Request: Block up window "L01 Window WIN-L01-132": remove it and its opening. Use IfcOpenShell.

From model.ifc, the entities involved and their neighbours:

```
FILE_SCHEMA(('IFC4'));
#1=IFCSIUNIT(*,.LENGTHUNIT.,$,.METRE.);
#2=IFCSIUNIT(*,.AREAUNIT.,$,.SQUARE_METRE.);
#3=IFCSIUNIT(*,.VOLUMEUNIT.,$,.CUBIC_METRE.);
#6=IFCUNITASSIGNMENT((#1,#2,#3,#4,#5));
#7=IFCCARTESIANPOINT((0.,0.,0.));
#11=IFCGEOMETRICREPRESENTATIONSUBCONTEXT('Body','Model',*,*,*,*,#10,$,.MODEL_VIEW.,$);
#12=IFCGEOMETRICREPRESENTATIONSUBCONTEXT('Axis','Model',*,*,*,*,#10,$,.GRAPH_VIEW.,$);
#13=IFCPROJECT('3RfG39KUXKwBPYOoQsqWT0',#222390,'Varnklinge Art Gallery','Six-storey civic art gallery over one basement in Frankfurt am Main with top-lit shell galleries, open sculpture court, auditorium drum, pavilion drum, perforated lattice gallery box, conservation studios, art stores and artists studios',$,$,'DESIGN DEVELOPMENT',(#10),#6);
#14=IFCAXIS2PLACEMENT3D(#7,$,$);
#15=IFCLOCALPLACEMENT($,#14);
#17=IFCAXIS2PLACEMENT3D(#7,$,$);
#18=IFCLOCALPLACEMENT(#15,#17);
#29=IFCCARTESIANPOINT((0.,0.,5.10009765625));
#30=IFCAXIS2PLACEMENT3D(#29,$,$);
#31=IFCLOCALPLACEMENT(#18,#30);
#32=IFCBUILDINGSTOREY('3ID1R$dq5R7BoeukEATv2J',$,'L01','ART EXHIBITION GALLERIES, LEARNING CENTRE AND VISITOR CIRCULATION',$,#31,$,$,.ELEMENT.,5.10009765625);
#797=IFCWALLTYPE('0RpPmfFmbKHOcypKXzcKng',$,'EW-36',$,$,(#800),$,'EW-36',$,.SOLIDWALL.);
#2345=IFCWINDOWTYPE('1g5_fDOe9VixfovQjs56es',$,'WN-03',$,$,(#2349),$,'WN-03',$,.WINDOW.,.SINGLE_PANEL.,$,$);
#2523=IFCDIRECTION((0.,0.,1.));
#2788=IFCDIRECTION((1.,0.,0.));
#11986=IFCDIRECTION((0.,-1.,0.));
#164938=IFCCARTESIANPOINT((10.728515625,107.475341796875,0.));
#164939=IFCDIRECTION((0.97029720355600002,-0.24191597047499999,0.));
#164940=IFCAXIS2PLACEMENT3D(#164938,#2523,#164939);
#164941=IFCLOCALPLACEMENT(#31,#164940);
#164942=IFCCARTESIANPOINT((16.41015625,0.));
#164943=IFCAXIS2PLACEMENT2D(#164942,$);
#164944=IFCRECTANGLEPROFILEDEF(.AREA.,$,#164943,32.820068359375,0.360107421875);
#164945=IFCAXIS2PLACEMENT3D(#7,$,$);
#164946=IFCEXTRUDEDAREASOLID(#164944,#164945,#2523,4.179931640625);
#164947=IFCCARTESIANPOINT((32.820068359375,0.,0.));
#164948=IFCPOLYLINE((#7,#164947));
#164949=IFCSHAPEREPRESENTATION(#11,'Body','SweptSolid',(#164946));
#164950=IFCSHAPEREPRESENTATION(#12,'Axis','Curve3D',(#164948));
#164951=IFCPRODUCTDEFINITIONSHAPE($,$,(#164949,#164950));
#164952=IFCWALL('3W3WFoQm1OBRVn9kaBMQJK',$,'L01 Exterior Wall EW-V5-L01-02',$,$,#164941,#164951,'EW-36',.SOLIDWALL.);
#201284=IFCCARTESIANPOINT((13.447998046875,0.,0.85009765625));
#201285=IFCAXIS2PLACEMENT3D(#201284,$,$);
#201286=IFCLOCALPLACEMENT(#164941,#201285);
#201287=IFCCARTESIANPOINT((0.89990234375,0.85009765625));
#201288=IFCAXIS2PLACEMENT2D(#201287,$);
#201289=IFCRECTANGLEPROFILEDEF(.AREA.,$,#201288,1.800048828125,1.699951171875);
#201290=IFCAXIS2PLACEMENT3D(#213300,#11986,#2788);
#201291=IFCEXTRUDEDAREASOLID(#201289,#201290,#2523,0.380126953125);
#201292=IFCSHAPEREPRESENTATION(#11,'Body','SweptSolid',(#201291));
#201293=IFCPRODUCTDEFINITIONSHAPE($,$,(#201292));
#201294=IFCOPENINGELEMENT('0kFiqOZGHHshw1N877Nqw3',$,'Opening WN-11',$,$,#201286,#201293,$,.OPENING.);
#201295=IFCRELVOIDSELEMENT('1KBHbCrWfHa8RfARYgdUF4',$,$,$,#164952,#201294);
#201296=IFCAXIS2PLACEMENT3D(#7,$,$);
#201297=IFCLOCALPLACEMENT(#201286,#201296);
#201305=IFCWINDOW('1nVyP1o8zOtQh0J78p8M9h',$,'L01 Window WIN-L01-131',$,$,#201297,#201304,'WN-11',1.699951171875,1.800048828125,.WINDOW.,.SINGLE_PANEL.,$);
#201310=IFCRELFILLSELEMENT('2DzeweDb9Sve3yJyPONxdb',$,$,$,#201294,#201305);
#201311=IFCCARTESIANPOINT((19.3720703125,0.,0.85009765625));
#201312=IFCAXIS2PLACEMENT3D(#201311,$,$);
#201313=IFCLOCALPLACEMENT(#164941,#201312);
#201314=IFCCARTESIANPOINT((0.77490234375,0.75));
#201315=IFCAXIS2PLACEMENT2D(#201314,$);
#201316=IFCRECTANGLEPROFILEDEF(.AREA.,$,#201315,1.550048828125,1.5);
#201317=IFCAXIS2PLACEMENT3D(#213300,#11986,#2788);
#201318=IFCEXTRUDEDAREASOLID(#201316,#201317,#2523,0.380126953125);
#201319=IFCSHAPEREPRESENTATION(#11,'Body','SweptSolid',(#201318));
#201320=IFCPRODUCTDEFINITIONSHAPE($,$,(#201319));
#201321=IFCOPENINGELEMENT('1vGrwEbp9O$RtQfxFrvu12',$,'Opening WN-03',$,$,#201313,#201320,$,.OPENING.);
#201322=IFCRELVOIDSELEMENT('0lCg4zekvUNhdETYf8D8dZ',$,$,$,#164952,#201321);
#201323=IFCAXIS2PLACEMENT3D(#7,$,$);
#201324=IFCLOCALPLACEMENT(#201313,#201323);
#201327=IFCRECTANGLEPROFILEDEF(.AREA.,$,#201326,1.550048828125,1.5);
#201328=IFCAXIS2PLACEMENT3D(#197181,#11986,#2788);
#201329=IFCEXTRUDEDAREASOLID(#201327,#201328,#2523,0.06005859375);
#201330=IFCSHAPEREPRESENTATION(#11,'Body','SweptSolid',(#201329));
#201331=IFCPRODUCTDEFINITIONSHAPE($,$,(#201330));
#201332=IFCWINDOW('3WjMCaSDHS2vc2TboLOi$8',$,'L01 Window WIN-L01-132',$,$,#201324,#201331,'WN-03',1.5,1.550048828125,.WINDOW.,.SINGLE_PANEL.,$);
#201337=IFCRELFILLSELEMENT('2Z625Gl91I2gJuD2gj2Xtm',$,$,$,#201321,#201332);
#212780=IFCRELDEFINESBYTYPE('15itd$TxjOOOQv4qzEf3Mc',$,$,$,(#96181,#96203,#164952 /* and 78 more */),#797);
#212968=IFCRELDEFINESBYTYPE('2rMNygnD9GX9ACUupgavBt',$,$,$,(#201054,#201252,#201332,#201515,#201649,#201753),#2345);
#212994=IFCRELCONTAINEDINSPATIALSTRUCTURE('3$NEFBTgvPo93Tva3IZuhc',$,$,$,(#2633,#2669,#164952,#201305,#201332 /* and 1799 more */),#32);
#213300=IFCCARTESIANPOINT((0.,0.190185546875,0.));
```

```python
import ifcopenshell
import ifcopenshell.api.feature
import ifcopenshell.api.root
import ifcopenshell.geom
import ifcopenshell.util.shape

model = ifcopenshell.open("model.ifc")
settings = ifcopenshell.geom.settings()


def volume(element):
    """Net volume in cubic metres, openings subtracted."""
    shape = ifcopenshell.geom.create_shape(settings, element)
    return ifcopenshell.util.shape.get_volume(shape.geometry)


window = model.by_guid("3WjMCaSDHS2vc2TboLOi$8")
opening = window.FillsVoids[0].RelatingOpeningElement
wall = opening.VoidsElements[0].RelatingBuildingElement
before = volume(wall)

ifcopenshell.api.root.remove_product(model, product=window)
ifcopenshell.api.feature.remove_feature(model, feature=opening)

after = volume(wall)

print(f"wall volume {before:.3f} -> {after:.3f} m3")

model.write("model_v2.ifc")
```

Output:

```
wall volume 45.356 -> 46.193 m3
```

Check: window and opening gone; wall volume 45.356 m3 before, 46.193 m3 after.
